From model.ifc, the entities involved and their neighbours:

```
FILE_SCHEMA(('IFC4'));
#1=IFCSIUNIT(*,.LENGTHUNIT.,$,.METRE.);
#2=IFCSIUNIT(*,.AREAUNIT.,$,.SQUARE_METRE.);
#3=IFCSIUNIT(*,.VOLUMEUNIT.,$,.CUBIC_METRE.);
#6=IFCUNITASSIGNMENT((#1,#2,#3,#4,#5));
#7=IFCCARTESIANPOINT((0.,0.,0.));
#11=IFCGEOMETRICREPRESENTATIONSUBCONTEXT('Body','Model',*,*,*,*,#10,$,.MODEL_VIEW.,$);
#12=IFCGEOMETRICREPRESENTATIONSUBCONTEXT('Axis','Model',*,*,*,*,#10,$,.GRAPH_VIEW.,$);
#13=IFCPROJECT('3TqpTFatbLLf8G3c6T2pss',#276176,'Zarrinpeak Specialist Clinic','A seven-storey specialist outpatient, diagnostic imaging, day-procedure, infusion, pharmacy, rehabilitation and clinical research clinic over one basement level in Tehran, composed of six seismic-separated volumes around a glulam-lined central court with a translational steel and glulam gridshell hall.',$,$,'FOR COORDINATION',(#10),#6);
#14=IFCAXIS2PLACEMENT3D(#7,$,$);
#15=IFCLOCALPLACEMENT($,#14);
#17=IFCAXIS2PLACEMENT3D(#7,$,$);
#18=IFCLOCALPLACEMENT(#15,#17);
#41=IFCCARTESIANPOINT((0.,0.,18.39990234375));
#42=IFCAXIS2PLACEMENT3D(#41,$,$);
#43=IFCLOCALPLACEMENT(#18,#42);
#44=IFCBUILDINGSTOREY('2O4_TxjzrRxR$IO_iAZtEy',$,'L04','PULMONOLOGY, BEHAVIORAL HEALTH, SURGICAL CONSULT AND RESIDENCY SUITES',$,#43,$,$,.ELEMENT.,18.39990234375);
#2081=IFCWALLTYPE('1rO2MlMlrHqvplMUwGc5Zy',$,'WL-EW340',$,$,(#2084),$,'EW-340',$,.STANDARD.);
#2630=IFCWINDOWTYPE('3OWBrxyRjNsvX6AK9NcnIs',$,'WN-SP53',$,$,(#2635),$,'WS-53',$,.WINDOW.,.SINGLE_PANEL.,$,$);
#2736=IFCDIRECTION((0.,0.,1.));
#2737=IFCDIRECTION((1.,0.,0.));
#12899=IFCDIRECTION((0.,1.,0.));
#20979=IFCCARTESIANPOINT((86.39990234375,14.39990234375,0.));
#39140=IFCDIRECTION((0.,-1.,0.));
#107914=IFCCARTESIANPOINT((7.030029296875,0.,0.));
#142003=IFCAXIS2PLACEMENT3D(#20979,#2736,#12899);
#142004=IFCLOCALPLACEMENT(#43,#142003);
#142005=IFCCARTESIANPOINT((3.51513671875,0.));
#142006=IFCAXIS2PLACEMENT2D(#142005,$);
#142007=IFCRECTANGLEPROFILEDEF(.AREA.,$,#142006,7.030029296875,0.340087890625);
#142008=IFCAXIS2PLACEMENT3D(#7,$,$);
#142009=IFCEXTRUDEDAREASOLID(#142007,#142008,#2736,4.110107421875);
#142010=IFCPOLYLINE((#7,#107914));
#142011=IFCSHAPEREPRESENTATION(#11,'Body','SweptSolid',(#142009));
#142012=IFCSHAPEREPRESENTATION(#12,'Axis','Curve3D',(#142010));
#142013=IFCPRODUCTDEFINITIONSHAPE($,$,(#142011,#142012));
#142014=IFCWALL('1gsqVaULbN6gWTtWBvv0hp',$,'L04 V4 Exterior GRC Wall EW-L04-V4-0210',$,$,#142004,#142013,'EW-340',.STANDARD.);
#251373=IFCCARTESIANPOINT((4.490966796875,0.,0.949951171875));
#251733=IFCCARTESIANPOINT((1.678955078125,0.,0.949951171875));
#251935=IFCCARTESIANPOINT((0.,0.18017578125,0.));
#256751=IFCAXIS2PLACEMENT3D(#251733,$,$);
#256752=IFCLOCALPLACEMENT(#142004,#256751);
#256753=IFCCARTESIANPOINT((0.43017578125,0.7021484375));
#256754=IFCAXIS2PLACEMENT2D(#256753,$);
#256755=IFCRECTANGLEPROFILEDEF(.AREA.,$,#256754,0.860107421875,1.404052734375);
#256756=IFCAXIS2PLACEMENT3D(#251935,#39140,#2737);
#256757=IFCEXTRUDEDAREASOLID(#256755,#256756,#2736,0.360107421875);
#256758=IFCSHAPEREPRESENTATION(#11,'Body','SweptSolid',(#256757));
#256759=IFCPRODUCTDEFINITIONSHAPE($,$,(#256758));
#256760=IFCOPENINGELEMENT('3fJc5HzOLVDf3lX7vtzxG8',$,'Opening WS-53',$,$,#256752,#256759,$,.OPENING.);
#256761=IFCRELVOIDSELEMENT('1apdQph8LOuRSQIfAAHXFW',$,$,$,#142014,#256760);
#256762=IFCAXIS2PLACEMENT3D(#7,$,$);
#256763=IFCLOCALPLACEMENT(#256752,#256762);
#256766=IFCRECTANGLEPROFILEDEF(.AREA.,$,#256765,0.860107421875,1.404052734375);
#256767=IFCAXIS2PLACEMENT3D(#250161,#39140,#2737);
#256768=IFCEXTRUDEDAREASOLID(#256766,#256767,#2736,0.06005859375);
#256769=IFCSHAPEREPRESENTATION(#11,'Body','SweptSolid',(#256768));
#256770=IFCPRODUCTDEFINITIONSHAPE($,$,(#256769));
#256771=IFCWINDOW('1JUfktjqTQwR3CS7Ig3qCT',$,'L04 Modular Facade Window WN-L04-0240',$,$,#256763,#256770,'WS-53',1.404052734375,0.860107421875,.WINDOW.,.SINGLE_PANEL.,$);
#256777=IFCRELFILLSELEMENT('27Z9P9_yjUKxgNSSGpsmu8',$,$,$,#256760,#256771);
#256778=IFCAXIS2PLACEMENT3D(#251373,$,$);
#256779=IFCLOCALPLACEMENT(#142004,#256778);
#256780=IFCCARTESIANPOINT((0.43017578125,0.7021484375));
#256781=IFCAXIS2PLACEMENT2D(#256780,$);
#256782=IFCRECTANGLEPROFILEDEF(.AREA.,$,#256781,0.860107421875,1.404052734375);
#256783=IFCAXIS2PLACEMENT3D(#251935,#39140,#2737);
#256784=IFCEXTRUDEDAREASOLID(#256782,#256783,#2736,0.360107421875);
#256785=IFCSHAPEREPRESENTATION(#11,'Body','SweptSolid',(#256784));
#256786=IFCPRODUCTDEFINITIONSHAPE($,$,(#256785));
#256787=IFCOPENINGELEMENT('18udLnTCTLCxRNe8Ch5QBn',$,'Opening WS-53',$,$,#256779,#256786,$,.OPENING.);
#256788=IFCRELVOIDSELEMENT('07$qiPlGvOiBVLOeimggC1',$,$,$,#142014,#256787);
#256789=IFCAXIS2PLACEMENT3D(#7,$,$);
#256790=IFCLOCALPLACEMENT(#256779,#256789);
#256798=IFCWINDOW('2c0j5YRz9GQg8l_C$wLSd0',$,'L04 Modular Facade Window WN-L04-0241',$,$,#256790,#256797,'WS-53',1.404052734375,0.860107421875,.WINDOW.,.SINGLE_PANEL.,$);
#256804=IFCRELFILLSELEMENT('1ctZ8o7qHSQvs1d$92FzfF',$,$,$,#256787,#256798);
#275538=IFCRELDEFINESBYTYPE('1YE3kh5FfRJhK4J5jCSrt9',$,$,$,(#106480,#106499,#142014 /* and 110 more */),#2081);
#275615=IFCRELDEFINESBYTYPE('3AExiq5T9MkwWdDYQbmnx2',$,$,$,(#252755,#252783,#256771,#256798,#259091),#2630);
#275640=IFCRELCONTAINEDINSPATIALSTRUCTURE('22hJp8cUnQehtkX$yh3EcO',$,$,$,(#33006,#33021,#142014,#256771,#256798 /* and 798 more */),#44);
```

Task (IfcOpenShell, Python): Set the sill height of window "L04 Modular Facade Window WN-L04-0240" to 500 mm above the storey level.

```python
import numpy as np
import ifcopenshell
import ifcopenshell.api.geometry
import ifcopenshell.geom
import ifcopenshell.util.element
import ifcopenshell.util.placement
import ifcopenshell.util.shape
import ifcopenshell.util.unit

model = ifcopenshell.open("model.ifc")
unit_scale = ifcopenshell.util.unit.calculate_unit_scale(model)

window = model.by_id(256771)
opening = window.FillsVoids[0].RelatingOpeningElement
storey = ifcopenshell.util.element.get_container(window, ifc_class="IfcBuildingStorey")
level = ifcopenshell.util.placement.get_local_placement(storey.ObjectPlacement)[2, 3]

# The opening's origin need not be at the sill, so measure its lowest point.
shape = ifcopenshell.geom.create_shape(ifcopenshell.geom.settings(), opening)
bottom = ifcopenshell.util.shape.get_shape_bottom_elevation(shape, shape.geometry) / unit_scale
dz = level + 0.5 - bottom

shift = np.array([0.0, 0.0, dz])
# The window is placed relative to its opening, so it follows when the opening moves.
matrix = ifcopenshell.util.placement.get_local_placement(opening.ObjectPlacement)
matrix[:3, 3] += shift
ifcopenshell.api.geometry.edit_object_placement(
    model, product=opening, matrix=matrix, is_si=False, should_transform_children=True
)

print(f"moved by {dz * unit_scale:+.3f} m")

model.write("model_rev.ifc")
```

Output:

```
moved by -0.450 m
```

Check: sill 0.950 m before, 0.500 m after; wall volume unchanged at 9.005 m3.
